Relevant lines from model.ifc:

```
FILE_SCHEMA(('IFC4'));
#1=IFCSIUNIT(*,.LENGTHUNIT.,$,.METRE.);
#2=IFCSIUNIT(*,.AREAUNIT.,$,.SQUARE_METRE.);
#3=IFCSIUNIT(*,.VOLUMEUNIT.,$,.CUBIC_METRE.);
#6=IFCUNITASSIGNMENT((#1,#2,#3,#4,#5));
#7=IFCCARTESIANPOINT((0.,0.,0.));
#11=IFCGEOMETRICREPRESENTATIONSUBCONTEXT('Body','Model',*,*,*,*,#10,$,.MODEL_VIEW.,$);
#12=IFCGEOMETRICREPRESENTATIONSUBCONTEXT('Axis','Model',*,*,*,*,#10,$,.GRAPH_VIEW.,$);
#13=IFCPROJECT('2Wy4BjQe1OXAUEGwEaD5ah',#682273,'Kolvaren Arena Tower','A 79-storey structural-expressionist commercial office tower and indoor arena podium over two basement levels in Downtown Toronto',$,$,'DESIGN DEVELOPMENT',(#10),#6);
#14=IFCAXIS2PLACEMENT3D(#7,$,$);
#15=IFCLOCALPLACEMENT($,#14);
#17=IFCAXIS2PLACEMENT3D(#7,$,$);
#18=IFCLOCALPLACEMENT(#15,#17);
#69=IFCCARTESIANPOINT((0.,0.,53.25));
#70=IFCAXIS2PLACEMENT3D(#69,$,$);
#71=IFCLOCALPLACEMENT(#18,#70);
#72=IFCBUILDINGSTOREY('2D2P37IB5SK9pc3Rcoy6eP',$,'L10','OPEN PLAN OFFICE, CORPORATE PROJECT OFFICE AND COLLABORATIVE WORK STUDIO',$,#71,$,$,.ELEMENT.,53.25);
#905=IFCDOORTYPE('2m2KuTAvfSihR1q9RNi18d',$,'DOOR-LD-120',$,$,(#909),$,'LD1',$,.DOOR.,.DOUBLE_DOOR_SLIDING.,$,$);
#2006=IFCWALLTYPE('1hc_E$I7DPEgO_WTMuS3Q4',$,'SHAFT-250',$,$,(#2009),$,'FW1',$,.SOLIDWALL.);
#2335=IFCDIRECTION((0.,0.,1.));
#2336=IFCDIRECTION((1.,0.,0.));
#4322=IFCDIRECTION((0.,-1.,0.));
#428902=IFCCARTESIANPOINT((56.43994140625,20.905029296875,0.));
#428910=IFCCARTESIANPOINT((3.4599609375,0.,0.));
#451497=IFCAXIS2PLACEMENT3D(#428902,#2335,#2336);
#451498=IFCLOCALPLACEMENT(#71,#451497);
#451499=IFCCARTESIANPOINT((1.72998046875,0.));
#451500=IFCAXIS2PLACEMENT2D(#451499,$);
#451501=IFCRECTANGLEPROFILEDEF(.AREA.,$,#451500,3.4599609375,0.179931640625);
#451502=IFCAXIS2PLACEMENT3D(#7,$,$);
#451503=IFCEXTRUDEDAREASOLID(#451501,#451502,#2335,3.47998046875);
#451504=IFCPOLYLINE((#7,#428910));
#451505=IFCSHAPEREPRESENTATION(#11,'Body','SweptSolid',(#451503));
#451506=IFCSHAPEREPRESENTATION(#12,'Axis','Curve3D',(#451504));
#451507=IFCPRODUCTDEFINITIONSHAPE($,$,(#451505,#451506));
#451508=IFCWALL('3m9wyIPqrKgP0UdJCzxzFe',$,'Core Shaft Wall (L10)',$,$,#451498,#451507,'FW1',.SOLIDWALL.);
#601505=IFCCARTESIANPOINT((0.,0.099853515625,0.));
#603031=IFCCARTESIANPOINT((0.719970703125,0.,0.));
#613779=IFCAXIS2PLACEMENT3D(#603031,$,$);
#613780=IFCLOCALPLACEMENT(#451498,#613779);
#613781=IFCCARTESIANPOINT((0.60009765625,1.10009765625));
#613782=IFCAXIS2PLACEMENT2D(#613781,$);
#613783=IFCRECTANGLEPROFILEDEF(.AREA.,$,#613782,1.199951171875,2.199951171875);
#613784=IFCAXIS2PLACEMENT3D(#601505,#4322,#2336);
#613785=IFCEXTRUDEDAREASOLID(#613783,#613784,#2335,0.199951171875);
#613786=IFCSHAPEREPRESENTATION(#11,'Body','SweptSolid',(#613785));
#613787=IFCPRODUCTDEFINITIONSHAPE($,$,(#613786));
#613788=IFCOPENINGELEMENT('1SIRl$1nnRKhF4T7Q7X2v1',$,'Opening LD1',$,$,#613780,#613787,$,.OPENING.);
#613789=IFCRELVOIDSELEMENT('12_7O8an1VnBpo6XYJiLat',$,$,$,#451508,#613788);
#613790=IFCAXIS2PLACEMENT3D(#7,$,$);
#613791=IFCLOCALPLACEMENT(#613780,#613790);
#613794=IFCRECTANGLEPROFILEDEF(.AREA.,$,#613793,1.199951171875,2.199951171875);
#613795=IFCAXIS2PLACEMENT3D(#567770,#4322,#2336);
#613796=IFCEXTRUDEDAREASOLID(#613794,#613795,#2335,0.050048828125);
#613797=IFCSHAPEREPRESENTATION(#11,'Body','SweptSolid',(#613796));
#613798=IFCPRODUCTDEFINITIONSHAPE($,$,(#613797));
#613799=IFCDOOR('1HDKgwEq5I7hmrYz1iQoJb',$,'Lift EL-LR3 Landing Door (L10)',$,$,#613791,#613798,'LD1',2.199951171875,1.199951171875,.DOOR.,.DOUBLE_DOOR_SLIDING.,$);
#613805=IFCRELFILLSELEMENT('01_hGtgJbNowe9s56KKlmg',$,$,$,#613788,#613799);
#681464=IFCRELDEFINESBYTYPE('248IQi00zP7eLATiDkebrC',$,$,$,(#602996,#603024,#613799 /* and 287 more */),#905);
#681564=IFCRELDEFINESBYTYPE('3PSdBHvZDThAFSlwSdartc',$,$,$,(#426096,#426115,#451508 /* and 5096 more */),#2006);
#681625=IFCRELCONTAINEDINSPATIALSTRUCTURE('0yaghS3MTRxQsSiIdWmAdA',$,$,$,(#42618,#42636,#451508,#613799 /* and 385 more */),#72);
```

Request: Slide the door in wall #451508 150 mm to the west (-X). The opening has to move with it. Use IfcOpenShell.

```python
import ifcopenshell
import ifcopenshell.api.geometry
import ifcopenshell.util.placement
import ifcopenshell.util.unit

model = ifcopenshell.open("model.ifc")
unit_scale = ifcopenshell.util.unit.calculate_unit_scale(model)

door = model.by_guid("1HDKgwEq5I7hmrYz1iQoJb")
opening = door.FillsVoids[0].RelatingOpeningElement
wall = opening.VoidsElements[0].RelatingBuildingElement

wall_matrix = ifcopenshell.util.placement.get_local_placement(wall.ObjectPlacement)
shift = wall_matrix[:3, 0] * -0.15 / unit_scale
before = ifcopenshell.util.placement.get_local_placement(door.ObjectPlacement)[:3, 3].copy()

# The door is placed relative to its opening, so it follows when the opening moves.
matrix = ifcopenshell.util.placement.get_local_placement(opening.ObjectPlacement)
matrix[:3, 3] += shift
ifcopenshell.api.geometry.edit_object_placement(
    model, product=opening, matrix=matrix, is_si=False, should_transform_children=True
)

after = ifcopenshell.util.placement.get_local_placement(door.ObjectPlacement)[:3, 3]
print("door moved by", (after - before).round(3) + 0.0)

model.write("model_edited.ifc")
```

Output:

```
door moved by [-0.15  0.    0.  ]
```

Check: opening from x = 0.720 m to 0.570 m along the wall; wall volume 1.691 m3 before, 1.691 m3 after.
